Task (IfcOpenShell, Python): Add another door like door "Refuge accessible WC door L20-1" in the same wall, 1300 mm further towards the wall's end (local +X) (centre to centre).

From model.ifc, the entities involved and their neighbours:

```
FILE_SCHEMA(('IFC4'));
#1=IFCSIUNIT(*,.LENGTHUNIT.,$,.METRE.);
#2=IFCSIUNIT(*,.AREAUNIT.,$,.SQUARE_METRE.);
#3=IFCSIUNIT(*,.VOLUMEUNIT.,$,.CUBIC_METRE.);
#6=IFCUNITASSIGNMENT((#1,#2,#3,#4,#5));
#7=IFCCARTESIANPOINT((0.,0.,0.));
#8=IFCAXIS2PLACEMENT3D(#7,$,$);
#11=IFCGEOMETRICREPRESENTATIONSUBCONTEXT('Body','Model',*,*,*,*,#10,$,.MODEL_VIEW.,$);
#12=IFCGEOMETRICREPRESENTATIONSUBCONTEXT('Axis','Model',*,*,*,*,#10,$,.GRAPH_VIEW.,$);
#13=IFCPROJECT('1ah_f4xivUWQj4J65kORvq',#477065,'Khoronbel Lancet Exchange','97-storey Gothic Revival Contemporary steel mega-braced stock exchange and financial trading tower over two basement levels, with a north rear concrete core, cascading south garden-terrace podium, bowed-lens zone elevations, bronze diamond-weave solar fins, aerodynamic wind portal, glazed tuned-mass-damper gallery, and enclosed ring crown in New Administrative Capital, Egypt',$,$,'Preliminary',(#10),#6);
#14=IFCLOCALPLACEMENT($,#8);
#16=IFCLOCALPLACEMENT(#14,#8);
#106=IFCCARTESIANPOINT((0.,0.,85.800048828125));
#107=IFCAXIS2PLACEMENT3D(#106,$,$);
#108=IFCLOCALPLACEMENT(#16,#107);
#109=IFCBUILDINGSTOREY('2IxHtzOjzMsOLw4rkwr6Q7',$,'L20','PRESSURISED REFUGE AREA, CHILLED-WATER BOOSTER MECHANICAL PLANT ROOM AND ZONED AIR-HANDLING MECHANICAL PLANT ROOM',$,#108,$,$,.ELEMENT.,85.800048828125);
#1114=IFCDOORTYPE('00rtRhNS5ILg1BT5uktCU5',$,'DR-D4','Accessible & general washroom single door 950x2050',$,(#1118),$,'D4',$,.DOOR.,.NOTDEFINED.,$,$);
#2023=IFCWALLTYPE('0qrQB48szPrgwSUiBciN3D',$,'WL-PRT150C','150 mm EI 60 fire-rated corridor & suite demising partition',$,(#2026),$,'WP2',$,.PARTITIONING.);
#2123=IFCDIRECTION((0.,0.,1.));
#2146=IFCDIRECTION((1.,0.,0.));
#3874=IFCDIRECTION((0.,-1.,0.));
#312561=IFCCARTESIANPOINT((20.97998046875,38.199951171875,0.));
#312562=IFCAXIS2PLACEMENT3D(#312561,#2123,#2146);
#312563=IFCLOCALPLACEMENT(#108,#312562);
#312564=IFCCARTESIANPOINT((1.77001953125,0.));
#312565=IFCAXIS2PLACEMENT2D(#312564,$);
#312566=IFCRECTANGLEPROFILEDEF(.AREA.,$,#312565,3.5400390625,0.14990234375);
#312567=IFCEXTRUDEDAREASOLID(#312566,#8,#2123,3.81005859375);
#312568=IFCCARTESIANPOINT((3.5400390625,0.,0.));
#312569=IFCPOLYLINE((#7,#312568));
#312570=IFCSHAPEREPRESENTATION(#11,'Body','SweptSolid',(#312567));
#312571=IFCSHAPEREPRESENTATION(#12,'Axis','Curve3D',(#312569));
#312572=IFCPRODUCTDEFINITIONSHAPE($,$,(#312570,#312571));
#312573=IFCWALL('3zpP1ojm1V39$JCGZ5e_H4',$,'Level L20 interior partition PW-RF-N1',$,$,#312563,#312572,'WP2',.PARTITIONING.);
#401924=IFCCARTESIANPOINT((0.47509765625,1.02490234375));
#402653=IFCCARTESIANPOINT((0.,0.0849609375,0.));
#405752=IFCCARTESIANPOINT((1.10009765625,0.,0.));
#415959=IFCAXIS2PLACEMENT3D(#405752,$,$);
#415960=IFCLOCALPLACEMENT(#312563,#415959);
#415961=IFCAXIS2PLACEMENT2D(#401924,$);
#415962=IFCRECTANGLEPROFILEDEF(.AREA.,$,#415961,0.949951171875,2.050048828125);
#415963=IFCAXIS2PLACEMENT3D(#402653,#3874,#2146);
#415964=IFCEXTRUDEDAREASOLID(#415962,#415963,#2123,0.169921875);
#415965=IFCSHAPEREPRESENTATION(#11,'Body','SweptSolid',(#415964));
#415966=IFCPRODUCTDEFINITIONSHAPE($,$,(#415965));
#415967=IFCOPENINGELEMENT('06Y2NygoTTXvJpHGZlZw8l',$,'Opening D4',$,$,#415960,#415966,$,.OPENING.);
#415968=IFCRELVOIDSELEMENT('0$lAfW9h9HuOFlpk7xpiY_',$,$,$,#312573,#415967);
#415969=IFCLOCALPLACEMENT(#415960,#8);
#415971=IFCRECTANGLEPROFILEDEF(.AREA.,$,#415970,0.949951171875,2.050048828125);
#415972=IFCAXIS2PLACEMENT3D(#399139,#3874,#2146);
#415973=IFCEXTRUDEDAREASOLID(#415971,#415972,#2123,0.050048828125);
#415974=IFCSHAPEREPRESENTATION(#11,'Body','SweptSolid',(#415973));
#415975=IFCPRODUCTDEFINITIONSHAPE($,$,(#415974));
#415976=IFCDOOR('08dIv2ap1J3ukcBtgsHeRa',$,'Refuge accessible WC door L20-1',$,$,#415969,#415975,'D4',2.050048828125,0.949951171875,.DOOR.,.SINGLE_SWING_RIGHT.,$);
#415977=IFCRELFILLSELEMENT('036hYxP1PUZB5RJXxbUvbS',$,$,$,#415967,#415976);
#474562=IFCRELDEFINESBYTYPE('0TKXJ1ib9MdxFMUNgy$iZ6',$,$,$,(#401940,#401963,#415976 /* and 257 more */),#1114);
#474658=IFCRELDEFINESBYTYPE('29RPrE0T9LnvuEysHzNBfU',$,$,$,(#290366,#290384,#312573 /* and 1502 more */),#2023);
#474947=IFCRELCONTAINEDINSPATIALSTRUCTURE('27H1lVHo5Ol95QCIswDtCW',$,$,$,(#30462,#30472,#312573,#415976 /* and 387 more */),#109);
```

```python
import ifcopenshell
import ifcopenshell.api.feature
import ifcopenshell.api.geometry
import ifcopenshell.api.root
import ifcopenshell.geom
import ifcopenshell.util.element
import ifcopenshell.util.placement
import ifcopenshell.util.shape
import ifcopenshell.util.unit

model = ifcopenshell.open("model.ifc")
unit_scale = ifcopenshell.util.unit.calculate_unit_scale(model)
settings = ifcopenshell.geom.settings()


def volume(element):
    """Net volume in cubic metres, openings subtracted."""
    shape = ifcopenshell.geom.create_shape(settings, element)
    return ifcopenshell.util.shape.get_volume(shape.geometry)


door = model.by_guid("08dIv2ap1J3ukcBtgsHeRa")
opening = door.FillsVoids[0].RelatingOpeningElement
wall = opening.VoidsElements[0].RelatingBuildingElement
before = volume(wall)
shift = ifcopenshell.util.placement.get_local_placement(wall.ObjectPlacement)[:3, 0] * 1.3 / unit_scale

# copy_class copies the void relationship, type, container and properties, but no geometry.
new_opening = ifcopenshell.api.root.copy_class(model, product=opening)
new_opening.Representation = ifcopenshell.util.element.copy_deep(
    model, opening.Representation, exclude=["IfcGeometricRepresentationContext", "IfcRepresentationMap"]
)
new_door = ifcopenshell.api.root.copy_class(model, product=door)
new_door.Representation = ifcopenshell.util.element.copy_deep(
    model, door.Representation, exclude=["IfcGeometricRepresentationContext", "IfcRepresentationMap"]
)
new_door.Tag = None
ifcopenshell.api.feature.add_filling(model, opening=new_opening, element=new_door)

for old, new in ((opening, new_opening), (door, new_door)):
    matrix = ifcopenshell.util.placement.get_local_placement(old.ObjectPlacement)
    matrix[:3, 3] += shift
    ifcopenshell.api.geometry.edit_object_placement(model, product=new, matrix=matrix, is_si=False)

after = volume(wall)

print(f"wall volume {before:.3f} -> {after:.3f} m3")

model.write("model_v2.ifc")
```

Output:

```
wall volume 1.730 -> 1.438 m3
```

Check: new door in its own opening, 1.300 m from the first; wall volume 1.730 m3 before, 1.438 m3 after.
